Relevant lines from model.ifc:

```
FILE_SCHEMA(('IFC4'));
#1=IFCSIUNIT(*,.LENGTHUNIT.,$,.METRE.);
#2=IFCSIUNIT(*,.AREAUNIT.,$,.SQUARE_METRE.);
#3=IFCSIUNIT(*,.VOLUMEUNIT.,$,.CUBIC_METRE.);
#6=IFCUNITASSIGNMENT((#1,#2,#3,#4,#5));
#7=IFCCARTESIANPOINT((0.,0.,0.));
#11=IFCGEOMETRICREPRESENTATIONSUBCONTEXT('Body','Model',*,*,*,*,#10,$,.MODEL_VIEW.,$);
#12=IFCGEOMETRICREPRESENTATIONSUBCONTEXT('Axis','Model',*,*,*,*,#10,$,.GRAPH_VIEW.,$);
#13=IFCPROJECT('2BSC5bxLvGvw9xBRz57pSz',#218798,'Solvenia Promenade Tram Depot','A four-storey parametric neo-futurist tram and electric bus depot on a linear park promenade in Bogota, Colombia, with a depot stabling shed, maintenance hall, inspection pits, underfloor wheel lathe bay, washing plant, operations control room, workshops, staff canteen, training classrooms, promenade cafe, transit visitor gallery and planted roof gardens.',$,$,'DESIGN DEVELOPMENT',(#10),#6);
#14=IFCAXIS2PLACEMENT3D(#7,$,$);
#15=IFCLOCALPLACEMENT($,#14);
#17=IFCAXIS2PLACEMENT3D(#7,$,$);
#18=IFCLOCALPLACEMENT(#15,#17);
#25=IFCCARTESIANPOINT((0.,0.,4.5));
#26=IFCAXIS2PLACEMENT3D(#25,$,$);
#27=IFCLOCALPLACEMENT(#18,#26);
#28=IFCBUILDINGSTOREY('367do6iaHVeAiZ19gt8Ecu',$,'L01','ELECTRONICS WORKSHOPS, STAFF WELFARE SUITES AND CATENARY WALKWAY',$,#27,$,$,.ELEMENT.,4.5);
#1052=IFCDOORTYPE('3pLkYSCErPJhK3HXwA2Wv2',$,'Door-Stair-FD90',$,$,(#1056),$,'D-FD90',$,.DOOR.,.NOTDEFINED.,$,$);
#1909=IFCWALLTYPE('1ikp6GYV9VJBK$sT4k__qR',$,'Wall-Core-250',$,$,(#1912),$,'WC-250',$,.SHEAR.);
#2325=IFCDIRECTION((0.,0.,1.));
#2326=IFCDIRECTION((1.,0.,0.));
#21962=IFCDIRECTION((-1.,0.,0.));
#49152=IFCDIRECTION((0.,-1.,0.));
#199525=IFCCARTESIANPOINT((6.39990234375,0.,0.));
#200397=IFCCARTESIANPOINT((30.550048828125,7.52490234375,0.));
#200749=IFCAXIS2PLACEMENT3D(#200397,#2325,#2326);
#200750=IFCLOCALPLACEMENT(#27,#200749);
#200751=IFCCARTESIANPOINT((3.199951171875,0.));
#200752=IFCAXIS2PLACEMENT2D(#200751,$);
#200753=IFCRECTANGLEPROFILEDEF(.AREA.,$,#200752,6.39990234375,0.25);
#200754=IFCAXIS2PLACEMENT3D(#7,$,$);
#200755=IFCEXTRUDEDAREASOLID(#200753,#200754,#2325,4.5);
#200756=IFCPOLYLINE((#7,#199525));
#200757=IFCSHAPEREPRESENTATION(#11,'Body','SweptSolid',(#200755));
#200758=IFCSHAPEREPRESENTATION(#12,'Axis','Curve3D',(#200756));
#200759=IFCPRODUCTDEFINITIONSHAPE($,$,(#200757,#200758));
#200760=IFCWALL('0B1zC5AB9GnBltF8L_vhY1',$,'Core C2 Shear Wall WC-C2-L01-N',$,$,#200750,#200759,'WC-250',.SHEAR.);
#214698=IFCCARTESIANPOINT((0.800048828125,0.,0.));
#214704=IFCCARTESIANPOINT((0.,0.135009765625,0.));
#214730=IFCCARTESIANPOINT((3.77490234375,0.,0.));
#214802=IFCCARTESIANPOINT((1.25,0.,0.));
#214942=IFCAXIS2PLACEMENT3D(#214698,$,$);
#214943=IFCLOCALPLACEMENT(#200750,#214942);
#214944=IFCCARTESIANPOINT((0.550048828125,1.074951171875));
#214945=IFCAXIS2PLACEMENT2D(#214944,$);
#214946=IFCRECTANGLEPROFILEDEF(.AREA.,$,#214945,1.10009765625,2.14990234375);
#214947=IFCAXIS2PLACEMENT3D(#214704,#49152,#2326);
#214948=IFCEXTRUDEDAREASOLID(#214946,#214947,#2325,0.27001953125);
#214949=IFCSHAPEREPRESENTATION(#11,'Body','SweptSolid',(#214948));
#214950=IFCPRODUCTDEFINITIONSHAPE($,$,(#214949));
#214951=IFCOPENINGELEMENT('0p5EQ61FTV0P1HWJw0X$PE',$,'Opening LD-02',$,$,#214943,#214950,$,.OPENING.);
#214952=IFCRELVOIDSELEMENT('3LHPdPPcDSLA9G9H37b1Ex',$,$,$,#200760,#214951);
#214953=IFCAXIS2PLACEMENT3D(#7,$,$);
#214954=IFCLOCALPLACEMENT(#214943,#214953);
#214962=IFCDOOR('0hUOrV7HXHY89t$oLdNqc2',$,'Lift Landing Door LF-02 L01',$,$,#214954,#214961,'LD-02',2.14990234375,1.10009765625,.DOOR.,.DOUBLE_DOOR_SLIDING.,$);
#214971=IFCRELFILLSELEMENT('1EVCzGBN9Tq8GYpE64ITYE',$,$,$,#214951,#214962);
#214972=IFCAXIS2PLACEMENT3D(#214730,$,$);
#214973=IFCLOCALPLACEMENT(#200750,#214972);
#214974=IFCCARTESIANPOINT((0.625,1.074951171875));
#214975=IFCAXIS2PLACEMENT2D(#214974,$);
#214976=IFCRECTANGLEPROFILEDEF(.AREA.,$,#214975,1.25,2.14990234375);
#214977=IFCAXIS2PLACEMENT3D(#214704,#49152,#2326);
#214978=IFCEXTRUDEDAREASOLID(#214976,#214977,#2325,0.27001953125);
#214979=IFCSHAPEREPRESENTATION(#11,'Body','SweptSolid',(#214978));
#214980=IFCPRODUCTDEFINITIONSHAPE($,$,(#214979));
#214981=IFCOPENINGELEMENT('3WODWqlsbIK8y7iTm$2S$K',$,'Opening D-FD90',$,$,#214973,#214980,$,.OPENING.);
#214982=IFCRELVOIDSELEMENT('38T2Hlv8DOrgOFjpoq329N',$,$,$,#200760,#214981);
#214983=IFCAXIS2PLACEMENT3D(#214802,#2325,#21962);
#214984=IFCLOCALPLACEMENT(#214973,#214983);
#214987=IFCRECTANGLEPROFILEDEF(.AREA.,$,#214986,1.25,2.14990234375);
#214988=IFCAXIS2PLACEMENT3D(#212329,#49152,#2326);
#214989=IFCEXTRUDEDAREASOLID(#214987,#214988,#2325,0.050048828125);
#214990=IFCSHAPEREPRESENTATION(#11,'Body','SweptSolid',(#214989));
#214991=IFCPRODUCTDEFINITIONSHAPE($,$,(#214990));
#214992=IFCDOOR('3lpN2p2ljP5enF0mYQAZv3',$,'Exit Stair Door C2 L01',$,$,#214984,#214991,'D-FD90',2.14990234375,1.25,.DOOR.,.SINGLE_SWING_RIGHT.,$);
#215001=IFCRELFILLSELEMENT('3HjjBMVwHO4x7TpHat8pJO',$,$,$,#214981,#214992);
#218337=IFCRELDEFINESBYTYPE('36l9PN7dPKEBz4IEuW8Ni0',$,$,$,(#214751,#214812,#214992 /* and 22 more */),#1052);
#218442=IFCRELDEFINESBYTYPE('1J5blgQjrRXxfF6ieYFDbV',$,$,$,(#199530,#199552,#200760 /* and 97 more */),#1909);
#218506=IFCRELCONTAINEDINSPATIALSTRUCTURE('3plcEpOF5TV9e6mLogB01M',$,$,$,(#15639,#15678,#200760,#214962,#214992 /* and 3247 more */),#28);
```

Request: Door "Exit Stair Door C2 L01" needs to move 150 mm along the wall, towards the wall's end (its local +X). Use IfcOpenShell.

```python
import ifcopenshell
import ifcopenshell.api.geometry
import ifcopenshell.util.placement
import ifcopenshell.util.unit

model = ifcopenshell.open("model.ifc")
unit_scale = ifcopenshell.util.unit.calculate_unit_scale(model)

door = model.by_guid("3lpN2p2ljP5enF0mYQAZv3")
opening = door.FillsVoids[0].RelatingOpeningElement
wall = opening.VoidsElements[0].RelatingBuildingElement

wall_matrix = ifcopenshell.util.placement.get_local_placement(wall.ObjectPlacement)
shift = wall_matrix[:3, 0] * 0.15 / unit_scale
before = ifcopenshell.util.placement.get_local_placement(door.ObjectPlacement)[:3, 3].copy()

# The door is placed relative to its opening, so it follows when the opening moves.
matrix = ifcopenshell.util.placement.get_local_placement(opening.ObjectPlacement)
matrix[:3, 3] += shift
ifcopenshell.api.geometry.edit_object_placement(
    model, product=opening, matrix=matrix, is_si=False, should_transform_children=True
)

after = ifcopenshell.util.placement.get_local_placement(door.ObjectPlacement)[:3, 3]
print("door moved by", (after - before).round(3) + 0.0)

model.write("model_edited.ifc")
```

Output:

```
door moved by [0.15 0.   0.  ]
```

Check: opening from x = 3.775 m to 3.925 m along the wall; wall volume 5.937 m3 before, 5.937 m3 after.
